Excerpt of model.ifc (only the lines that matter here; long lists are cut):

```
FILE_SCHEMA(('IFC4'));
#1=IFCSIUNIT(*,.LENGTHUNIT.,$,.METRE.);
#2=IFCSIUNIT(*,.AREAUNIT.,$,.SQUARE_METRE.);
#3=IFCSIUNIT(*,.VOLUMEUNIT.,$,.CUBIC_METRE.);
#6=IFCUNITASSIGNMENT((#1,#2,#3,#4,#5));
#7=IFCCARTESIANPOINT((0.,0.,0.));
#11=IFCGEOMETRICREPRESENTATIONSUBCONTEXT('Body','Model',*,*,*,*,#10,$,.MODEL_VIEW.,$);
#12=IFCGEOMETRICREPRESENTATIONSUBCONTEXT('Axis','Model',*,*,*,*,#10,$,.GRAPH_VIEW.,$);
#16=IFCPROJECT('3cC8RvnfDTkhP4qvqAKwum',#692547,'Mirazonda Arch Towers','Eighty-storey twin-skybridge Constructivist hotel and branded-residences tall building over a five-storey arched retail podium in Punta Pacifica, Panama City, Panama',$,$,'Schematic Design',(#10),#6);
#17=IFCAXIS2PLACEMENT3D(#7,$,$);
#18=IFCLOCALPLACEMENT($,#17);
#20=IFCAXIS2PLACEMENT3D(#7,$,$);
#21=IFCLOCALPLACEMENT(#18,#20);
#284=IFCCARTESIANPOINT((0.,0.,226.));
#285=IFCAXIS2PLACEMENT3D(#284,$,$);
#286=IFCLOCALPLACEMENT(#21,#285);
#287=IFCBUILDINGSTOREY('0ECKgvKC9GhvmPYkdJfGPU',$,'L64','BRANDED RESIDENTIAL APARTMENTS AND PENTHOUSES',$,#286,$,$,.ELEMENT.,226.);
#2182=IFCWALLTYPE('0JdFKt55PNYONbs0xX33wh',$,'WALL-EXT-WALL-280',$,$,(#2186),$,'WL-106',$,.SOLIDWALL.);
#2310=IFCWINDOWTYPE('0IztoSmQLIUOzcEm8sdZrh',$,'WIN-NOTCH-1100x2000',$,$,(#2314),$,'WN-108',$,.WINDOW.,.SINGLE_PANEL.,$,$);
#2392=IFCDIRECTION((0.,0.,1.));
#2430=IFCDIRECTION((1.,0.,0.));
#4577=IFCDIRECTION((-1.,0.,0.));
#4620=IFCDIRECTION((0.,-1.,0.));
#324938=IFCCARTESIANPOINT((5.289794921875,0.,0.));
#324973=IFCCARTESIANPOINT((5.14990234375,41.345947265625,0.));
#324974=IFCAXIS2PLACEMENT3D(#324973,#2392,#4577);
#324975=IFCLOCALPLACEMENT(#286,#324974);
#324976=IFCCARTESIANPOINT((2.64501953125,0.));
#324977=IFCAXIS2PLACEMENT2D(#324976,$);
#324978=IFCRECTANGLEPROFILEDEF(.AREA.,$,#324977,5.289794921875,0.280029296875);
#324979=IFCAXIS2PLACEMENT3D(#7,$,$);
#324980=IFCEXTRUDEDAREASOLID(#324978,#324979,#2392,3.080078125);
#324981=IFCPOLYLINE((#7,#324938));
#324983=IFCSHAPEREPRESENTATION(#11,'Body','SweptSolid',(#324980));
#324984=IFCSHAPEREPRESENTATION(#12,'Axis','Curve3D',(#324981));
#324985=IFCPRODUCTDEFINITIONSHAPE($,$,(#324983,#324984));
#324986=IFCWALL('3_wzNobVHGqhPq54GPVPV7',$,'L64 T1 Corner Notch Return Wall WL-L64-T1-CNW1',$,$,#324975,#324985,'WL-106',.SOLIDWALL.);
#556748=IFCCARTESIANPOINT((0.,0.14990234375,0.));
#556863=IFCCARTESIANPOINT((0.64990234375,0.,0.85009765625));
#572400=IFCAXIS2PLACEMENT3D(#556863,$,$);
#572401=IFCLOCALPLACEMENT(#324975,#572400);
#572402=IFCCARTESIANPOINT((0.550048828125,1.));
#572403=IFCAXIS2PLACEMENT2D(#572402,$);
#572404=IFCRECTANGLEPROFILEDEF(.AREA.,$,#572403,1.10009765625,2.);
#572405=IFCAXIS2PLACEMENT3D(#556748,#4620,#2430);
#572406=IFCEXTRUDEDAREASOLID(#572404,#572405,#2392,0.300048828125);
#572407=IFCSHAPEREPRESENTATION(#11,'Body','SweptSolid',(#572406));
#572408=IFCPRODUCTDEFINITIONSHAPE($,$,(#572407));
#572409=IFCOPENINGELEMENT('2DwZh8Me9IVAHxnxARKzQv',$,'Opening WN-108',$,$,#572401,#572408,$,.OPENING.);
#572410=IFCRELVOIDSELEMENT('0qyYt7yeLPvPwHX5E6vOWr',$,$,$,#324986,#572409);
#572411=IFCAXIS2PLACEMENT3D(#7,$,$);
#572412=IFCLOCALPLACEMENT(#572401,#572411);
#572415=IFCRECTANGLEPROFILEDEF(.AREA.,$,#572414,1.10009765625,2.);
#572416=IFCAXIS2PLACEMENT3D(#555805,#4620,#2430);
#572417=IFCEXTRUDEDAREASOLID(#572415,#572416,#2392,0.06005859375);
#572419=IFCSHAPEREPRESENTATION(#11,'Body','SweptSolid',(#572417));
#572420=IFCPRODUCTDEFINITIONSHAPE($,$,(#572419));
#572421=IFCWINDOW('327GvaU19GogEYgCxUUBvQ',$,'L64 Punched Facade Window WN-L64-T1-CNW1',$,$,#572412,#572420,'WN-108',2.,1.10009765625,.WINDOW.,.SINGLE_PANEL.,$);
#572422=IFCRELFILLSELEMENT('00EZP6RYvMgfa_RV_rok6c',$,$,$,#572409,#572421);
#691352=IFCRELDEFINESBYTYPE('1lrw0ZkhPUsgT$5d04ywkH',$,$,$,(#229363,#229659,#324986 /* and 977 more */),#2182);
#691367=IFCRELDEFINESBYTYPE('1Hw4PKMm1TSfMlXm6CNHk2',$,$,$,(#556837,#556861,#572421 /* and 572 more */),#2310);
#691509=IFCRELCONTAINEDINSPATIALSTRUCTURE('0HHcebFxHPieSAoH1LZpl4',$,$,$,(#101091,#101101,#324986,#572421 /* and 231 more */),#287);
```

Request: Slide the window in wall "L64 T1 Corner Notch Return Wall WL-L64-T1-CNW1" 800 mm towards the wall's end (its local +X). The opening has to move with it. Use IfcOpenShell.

```python
import ifcopenshell
import ifcopenshell.api.geometry
import ifcopenshell.util.placement
import ifcopenshell.util.unit

model = ifcopenshell.open("model.ifc")
unit_scale = ifcopenshell.util.unit.calculate_unit_scale(model)

window = model.by_guid("327GvaU19GogEYgCxUUBvQ")
opening = window.FillsVoids[0].RelatingOpeningElement
wall = opening.VoidsElements[0].RelatingBuildingElement

wall_matrix = ifcopenshell.util.placement.get_local_placement(wall.ObjectPlacement)
shift = wall_matrix[:3, 0] * 0.8 / unit_scale
before = ifcopenshell.util.placement.get_local_placement(window.ObjectPlacement)[:3, 3].copy()

# The window is placed relative to its opening, so it follows when the opening moves.
matrix = ifcopenshell.util.placement.get_local_placement(opening.ObjectPlacement)
matrix[:3, 3] += shift
ifcopenshell.api.geometry.edit_object_placement(
    model, product=opening, matrix=matrix, is_si=False, should_transform_children=True
)

after = ifcopenshell.util.placement.get_local_placement(window.ObjectPlacement)[:3, 3]
print("window moved by", (after - before).round(3) + 0.0)

model.write("model_v2.ifc")
```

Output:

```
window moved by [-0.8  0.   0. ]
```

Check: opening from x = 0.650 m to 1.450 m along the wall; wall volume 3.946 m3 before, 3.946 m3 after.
